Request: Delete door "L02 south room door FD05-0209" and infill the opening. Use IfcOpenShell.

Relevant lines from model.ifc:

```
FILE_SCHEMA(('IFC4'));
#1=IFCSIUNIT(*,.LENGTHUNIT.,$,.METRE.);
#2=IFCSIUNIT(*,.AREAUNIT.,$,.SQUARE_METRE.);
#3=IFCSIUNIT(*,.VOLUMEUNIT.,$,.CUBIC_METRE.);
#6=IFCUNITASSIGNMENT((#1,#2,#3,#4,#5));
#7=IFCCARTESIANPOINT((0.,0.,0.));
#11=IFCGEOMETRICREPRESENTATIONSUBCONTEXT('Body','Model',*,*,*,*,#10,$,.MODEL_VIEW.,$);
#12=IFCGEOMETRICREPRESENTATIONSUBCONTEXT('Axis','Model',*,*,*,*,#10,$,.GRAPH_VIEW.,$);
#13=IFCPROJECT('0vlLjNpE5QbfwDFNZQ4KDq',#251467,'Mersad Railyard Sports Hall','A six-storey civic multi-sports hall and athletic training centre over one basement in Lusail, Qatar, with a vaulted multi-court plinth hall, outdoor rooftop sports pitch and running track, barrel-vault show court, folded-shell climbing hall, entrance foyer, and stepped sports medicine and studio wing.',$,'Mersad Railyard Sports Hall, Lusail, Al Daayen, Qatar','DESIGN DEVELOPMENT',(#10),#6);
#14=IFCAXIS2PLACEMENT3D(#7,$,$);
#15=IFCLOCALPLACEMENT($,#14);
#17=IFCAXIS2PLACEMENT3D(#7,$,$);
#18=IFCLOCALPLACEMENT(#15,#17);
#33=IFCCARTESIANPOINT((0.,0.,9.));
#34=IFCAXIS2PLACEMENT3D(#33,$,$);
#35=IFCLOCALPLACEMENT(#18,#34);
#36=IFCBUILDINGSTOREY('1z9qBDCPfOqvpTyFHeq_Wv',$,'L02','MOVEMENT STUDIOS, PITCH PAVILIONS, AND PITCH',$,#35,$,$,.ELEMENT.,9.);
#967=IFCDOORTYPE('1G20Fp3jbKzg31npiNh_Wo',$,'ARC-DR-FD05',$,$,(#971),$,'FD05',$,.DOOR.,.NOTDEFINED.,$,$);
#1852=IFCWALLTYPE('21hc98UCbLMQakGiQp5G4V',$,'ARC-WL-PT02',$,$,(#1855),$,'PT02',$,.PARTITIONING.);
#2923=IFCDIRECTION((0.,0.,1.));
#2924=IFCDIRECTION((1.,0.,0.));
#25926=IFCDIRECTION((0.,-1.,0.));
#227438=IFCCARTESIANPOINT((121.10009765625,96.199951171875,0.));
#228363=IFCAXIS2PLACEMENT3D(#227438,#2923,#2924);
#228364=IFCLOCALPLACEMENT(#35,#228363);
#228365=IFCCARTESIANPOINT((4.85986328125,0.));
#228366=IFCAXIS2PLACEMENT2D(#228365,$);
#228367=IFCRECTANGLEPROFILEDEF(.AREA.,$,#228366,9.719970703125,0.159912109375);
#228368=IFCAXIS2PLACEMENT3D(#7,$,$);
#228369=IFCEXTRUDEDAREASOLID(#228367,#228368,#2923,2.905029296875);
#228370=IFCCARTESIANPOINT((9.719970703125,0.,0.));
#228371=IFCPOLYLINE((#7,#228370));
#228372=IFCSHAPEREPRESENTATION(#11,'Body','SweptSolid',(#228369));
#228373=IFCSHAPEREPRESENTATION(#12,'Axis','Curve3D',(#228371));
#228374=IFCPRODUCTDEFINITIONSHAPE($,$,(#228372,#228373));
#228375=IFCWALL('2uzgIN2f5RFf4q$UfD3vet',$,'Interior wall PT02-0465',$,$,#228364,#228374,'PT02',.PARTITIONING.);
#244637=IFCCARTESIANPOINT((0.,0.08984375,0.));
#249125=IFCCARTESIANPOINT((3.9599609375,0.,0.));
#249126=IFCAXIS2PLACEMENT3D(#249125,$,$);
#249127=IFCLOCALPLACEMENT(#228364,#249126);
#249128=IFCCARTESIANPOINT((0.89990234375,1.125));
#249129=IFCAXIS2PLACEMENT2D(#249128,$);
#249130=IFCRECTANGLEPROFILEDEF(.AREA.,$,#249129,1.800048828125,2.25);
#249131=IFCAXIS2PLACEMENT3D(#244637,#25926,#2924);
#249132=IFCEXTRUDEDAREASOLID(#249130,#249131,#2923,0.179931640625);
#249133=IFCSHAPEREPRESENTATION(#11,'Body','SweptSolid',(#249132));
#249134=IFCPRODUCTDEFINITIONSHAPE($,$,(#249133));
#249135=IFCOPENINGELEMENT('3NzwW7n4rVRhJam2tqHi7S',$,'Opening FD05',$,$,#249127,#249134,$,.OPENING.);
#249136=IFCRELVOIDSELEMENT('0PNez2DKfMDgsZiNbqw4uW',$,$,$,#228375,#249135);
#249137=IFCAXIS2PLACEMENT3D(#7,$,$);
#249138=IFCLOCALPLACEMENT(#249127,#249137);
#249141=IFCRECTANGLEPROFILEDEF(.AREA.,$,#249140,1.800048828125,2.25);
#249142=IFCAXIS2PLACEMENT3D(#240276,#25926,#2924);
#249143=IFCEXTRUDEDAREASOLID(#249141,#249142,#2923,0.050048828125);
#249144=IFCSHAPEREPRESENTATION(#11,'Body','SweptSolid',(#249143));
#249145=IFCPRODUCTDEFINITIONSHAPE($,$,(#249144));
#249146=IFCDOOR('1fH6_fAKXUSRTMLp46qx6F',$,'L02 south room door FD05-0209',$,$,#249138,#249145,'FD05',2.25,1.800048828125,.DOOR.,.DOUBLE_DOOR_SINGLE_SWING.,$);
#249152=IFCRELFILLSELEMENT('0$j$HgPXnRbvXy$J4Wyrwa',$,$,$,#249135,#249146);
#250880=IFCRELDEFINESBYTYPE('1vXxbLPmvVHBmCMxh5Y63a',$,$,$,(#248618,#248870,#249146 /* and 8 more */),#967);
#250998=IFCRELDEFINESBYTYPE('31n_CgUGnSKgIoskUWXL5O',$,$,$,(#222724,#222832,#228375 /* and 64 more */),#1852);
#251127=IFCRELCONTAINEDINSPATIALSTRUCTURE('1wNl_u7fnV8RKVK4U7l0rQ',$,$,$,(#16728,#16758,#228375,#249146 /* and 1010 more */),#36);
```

```python
import ifcopenshell
import ifcopenshell.api.feature
import ifcopenshell.api.root
import ifcopenshell.geom
import ifcopenshell.util.shape

model = ifcopenshell.open("model.ifc")
settings = ifcopenshell.geom.settings()


def volume(element):
    """Net volume in cubic metres, openings subtracted."""
    shape = ifcopenshell.geom.create_shape(settings, element)
    return ifcopenshell.util.shape.get_volume(shape.geometry)


door = model.by_guid("1fH6_fAKXUSRTMLp46qx6F")
opening = door.FillsVoids[0].RelatingOpeningElement
wall = opening.VoidsElements[0].RelatingBuildingElement
before = volume(wall)

ifcopenshell.api.root.remove_product(model, product=door)
ifcopenshell.api.feature.remove_feature(model, feature=opening)

after = volume(wall)

print(f"wall volume {before:.3f} -> {after:.3f} m3")

model.write("model-out.ifc")
```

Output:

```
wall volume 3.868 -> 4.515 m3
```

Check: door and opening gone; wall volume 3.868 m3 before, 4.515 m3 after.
